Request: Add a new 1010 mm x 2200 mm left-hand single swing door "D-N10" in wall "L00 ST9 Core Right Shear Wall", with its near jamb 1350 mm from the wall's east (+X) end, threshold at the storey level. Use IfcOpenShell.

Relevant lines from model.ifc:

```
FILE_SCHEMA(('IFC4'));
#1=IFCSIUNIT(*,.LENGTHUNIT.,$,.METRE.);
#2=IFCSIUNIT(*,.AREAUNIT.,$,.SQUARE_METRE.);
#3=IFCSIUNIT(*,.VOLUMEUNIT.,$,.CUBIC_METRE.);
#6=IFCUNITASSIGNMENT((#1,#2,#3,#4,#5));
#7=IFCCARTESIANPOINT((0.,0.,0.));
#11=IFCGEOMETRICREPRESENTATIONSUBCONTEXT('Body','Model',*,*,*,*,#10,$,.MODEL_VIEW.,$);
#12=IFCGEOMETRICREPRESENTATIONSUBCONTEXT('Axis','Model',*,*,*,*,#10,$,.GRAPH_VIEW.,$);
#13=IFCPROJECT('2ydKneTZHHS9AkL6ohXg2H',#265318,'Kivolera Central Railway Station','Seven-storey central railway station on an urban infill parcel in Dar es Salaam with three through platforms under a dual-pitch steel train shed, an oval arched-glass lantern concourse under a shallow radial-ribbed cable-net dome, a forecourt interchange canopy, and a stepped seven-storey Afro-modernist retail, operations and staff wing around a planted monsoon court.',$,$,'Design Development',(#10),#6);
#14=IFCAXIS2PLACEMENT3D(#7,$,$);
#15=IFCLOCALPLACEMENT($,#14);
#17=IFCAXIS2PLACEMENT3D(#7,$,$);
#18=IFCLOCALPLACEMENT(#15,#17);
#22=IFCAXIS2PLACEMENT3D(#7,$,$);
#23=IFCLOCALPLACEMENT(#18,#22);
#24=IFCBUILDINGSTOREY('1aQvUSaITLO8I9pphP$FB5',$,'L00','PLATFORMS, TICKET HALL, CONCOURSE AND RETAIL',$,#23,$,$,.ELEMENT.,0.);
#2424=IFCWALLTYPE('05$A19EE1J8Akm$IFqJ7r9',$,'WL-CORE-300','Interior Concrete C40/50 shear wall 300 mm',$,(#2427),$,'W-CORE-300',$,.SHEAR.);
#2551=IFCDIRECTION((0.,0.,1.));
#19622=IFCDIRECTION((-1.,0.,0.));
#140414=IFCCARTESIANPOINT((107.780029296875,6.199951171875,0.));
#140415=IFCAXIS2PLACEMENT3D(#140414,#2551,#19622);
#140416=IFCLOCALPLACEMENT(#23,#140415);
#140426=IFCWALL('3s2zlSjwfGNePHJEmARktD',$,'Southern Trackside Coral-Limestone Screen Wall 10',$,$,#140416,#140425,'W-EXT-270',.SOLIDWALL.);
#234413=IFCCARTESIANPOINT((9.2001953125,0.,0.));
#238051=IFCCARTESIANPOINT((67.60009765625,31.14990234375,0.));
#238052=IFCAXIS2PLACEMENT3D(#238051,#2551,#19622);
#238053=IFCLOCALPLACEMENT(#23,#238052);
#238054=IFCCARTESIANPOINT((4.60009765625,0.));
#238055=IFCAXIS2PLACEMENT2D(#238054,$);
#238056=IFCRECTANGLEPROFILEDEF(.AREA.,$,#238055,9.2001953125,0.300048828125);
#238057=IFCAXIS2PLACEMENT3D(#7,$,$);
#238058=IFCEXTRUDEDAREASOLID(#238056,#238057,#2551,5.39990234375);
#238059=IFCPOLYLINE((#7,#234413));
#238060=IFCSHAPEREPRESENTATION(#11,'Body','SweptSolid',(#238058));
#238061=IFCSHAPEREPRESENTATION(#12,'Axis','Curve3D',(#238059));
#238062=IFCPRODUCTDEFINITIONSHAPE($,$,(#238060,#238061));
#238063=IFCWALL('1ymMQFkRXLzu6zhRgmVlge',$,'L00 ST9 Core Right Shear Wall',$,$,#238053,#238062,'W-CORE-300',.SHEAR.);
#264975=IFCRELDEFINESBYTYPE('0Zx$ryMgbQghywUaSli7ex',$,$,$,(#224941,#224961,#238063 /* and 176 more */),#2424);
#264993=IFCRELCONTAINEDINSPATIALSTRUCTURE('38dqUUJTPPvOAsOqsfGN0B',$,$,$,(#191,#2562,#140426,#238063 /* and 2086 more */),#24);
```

```python
import numpy as np
import ifcopenshell
import ifcopenshell.api.feature
import ifcopenshell.api.geometry
import ifcopenshell.api.root
import ifcopenshell.api.spatial
import ifcopenshell.geom
import ifcopenshell.util.element
import ifcopenshell.util.placement
import ifcopenshell.util.representation
import ifcopenshell.util.shape
import ifcopenshell.util.unit

model = ifcopenshell.open("model.ifc")
unit_scale = ifcopenshell.util.unit.calculate_unit_scale(model)
settings = ifcopenshell.geom.settings()


def volume(element):
    """Net volume in cubic metres, openings subtracted."""
    shape = ifcopenshell.geom.create_shape(settings, element)
    return ifcopenshell.util.shape.get_volume(shape.geometry)


wall = model.by_guid("1ymMQFkRXLzu6zhRgmVlge")
storey = ifcopenshell.util.element.get_container(wall, ifc_class="IfcBuildingStorey")
context = ifcopenshell.util.representation.get_context(model, "Model", "Body", "MODEL_VIEW")
before = volume(wall)

width, height, from_end, sill = 1.01, 2.2, 1.35, 0.0  # metres

# The wall runs along its own X axis, and the end named is its -X end.
wall_shape = ifcopenshell.geom.create_shape(settings, wall)
x, y, z = ifcopenshell.util.shape.get_vertices(wall_shape.geometry).T
start = x.min() + from_end
face, thickness = float(y.min()), float(y.max() - y.min())
wall_matrix = ifcopenshell.util.placement.get_local_placement(wall.ObjectPlacement)
level = ifcopenshell.util.placement.get_local_placement(storey.ObjectPlacement)[2, 3]


def in_wall(x, y):
    """Placement at x, y metres in the wall's axes, at sill height."""
    matrix = wall_matrix.copy()
    matrix[:, 3] = wall_matrix @ np.array([x / unit_scale, y / unit_scale, 0.0, 1.0])
    matrix[2, 3] = level + sill / unit_scale
    return matrix


# Opening: a box that overshoots both wall faces by 50 mm.
opening = ifcopenshell.api.root.create_entity(model, ifc_class="IfcOpeningElement", predefined_type="OPENING")
box = ifcopenshell.api.geometry.add_wall_representation(
    model, context=context, length=width, height=height, thickness=thickness + 0.1
)
ifcopenshell.api.geometry.assign_representation(model, product=opening, representation=box)
ifcopenshell.api.geometry.edit_object_placement(model, product=opening, matrix=in_wall(start, face - 0.05), is_si=False)
ifcopenshell.api.feature.add_feature(model, feature=opening, element=wall)

door = ifcopenshell.api.root.create_entity(model, ifc_class="IfcDoor", name="D-N10", predefined_type="DOOR")
door.OverallWidth, door.OverallHeight = width / unit_scale, height / unit_scale
door.OperationType = "SINGLE_SWING_LEFT"
body = ifcopenshell.api.geometry.add_door_representation(
    model,
    context=context,
    overall_width=door.OverallWidth,
    overall_height=door.OverallHeight,
    operation_type="SINGLE_SWING_LEFT",
    lining_properties={"LiningDepth": thickness / unit_scale, "ThresholdDepth": thickness / unit_scale},
)
ifcopenshell.api.geometry.assign_representation(model, product=door, representation=body)
ifcopenshell.api.spatial.assign_container(model, products=[door], relating_structure=storey)
ifcopenshell.api.feature.add_filling(model, opening=opening, element=door)

# The lining spans the wall, so the door starts at the wall face.
ifcopenshell.api.geometry.edit_object_placement(model, product=door, matrix=in_wall(start, face), is_si=False)

after = volume(wall)

print(f"wall volume {before:.3f} -> {after:.3f} m3")

model.write("model_edited.ifc")
```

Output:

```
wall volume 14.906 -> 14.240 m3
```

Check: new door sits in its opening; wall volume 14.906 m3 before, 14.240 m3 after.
